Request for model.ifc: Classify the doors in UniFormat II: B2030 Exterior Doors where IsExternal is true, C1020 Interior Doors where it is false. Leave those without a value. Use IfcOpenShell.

First a look at what the model holds.

```python
import ifcopenshell
import ifcopenshell.util.element

model = ifcopenshell.open("model.ifc")
print(model.schema)
print("classifications:", [c.Name for c in model.by_type("IfcClassification")])
values = [ifcopenshell.util.element.get_pset(e, "Pset_DoorCommon", "IsExternal") for e in model.by_type("IfcDoor")]
for value in (True, False, None):
    print("IsExternal", value, values.count(value))
```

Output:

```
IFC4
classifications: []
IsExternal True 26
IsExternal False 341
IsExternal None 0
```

```python
import ifcopenshell
import ifcopenshell.api.classification
import ifcopenshell.util.element

model = ifcopenshell.open("model.ifc")

system = ifcopenshell.api.classification.add_classification(model, classification="UniFormat II")

doors = model.by_type("IfcDoor")
external = {e: ifcopenshell.util.element.get_pset(e, "Pset_DoorCommon", "IsExternal") for e in doors}
for flag, code, name in ((True, "B2030", "Exterior Doors"), (False, "C1020", "Interior Doors")):
    products = [e for e in doors if external[e] is flag]
    ifcopenshell.api.classification.add_reference(
        model, products=products, classification=system, identification=code, name=name
    )
    print(code, len(products))

model.write("model_edited.ifc")
```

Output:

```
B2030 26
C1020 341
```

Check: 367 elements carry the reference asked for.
